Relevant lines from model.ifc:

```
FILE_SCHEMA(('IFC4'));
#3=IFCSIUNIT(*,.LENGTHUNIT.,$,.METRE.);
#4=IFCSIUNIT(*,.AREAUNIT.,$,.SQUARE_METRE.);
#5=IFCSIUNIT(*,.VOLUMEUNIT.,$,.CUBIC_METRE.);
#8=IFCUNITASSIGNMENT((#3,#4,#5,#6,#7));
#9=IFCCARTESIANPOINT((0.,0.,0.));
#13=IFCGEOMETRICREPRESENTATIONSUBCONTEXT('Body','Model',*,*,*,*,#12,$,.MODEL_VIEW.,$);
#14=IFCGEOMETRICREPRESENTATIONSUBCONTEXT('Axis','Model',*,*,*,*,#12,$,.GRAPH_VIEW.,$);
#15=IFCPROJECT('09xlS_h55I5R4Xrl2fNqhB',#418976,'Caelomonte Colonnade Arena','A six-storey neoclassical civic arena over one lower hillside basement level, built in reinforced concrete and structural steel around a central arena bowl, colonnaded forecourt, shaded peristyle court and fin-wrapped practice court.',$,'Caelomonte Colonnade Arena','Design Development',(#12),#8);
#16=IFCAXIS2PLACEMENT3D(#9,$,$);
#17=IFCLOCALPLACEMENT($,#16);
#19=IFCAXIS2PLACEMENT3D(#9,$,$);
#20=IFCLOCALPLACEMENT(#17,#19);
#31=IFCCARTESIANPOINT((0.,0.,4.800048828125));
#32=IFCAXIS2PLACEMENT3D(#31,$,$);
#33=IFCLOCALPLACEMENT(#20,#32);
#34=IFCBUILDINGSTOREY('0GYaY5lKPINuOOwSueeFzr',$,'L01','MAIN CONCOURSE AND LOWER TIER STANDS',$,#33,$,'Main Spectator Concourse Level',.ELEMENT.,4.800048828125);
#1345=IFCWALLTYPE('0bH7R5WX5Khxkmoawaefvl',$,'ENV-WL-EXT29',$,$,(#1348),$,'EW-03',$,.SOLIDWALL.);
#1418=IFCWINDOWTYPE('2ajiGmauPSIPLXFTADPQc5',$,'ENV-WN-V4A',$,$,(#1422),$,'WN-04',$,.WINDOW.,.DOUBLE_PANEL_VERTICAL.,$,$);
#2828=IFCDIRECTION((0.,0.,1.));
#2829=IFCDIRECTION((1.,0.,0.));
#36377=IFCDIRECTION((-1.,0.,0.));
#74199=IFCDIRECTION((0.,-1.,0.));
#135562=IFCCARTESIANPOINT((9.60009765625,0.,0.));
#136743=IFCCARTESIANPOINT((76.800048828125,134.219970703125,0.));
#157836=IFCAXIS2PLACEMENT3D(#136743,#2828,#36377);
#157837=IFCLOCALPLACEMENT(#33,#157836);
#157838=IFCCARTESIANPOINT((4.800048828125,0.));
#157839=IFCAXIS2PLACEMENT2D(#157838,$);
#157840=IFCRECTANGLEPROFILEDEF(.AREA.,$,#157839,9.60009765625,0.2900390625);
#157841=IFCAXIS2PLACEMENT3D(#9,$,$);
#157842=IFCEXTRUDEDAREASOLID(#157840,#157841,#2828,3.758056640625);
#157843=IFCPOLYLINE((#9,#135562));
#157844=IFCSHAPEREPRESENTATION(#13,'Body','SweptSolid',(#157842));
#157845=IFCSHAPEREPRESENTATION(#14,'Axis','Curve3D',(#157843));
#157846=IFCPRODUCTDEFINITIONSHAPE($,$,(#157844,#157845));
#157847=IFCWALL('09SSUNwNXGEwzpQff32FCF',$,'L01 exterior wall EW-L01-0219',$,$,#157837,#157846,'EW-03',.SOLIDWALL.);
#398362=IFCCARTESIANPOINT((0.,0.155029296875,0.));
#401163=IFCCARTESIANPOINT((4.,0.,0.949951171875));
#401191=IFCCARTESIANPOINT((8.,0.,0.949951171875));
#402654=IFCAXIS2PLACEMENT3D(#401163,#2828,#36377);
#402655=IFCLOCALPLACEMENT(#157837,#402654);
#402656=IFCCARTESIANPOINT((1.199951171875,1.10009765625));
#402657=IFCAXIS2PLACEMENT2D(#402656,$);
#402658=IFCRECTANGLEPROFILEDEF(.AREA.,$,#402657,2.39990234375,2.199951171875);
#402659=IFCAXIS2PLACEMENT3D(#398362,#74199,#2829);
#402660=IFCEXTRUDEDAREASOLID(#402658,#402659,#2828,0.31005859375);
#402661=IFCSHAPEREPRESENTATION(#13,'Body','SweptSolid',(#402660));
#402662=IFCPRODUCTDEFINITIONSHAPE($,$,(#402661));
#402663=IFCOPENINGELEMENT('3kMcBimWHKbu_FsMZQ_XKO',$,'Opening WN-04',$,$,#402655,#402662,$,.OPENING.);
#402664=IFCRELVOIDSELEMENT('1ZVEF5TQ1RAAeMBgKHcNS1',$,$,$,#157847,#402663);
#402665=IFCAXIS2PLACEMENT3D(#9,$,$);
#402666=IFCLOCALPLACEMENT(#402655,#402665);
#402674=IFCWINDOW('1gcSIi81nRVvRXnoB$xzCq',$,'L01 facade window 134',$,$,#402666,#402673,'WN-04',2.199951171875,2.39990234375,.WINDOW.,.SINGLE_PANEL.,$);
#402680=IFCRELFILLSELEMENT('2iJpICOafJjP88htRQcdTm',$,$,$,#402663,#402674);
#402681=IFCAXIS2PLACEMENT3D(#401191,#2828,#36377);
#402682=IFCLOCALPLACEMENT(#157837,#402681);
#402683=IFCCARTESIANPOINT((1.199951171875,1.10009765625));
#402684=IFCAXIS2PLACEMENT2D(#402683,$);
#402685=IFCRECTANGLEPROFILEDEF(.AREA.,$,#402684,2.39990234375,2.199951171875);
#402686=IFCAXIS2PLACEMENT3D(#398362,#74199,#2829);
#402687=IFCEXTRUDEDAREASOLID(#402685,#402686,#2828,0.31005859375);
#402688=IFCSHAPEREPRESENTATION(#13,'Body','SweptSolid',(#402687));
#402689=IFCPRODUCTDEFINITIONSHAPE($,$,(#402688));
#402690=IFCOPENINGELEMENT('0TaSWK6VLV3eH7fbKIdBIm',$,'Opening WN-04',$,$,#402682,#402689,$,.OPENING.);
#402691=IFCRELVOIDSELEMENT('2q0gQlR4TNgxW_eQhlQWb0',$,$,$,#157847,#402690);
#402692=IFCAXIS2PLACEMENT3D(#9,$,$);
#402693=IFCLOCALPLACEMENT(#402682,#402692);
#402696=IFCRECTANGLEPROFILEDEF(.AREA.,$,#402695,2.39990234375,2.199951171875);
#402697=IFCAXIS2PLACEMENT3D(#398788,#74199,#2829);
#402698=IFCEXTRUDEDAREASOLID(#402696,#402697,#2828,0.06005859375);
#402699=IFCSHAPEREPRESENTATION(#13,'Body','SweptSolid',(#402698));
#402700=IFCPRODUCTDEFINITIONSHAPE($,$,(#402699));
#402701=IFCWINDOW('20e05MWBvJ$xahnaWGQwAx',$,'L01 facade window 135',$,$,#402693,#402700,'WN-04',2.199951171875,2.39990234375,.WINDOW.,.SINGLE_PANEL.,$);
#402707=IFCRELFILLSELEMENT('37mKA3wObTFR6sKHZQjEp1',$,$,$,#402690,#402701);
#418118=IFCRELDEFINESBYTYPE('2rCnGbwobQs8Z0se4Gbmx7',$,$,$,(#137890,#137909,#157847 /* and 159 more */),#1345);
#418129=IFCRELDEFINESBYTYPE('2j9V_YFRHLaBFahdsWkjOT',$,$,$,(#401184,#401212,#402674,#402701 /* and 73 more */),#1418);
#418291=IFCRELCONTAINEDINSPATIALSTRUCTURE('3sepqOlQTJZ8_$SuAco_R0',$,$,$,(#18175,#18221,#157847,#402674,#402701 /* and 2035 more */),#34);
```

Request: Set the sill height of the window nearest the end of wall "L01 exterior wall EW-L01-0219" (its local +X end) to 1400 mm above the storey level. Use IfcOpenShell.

```python
import numpy as np
import ifcopenshell
import ifcopenshell.api.geometry
import ifcopenshell.geom
import ifcopenshell.util.element
import ifcopenshell.util.placement
import ifcopenshell.util.shape
import ifcopenshell.util.unit

model = ifcopenshell.open("model.ifc")
unit_scale = ifcopenshell.util.unit.calculate_unit_scale(model)

window = model.by_guid("20e05MWBvJ$xahnaWGQwAx")
opening = window.FillsVoids[0].RelatingOpeningElement
storey = ifcopenshell.util.element.get_container(window, ifc_class="IfcBuildingStorey")
level = ifcopenshell.util.placement.get_local_placement(storey.ObjectPlacement)[2, 3]

# The opening's origin need not be at the sill, so measure its lowest point.
shape = ifcopenshell.geom.create_shape(ifcopenshell.geom.settings(), opening)
bottom = ifcopenshell.util.shape.get_shape_bottom_elevation(shape, shape.geometry) / unit_scale
dz = level + 1.4 / unit_scale - bottom

shift = np.array([0.0, 0.0, dz])
# The window is placed relative to its opening, so it follows when the opening moves.
matrix = ifcopenshell.util.placement.get_local_placement(opening.ObjectPlacement)
matrix[:3, 3] += shift
ifcopenshell.api.geometry.edit_object_placement(
    model, product=opening, matrix=matrix, is_si=False, should_transform_children=True
)

print(f"moved by {dz * unit_scale:+.3f} m")

model.write("model_v2.ifc")
```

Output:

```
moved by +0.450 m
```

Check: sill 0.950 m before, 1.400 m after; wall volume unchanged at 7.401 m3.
